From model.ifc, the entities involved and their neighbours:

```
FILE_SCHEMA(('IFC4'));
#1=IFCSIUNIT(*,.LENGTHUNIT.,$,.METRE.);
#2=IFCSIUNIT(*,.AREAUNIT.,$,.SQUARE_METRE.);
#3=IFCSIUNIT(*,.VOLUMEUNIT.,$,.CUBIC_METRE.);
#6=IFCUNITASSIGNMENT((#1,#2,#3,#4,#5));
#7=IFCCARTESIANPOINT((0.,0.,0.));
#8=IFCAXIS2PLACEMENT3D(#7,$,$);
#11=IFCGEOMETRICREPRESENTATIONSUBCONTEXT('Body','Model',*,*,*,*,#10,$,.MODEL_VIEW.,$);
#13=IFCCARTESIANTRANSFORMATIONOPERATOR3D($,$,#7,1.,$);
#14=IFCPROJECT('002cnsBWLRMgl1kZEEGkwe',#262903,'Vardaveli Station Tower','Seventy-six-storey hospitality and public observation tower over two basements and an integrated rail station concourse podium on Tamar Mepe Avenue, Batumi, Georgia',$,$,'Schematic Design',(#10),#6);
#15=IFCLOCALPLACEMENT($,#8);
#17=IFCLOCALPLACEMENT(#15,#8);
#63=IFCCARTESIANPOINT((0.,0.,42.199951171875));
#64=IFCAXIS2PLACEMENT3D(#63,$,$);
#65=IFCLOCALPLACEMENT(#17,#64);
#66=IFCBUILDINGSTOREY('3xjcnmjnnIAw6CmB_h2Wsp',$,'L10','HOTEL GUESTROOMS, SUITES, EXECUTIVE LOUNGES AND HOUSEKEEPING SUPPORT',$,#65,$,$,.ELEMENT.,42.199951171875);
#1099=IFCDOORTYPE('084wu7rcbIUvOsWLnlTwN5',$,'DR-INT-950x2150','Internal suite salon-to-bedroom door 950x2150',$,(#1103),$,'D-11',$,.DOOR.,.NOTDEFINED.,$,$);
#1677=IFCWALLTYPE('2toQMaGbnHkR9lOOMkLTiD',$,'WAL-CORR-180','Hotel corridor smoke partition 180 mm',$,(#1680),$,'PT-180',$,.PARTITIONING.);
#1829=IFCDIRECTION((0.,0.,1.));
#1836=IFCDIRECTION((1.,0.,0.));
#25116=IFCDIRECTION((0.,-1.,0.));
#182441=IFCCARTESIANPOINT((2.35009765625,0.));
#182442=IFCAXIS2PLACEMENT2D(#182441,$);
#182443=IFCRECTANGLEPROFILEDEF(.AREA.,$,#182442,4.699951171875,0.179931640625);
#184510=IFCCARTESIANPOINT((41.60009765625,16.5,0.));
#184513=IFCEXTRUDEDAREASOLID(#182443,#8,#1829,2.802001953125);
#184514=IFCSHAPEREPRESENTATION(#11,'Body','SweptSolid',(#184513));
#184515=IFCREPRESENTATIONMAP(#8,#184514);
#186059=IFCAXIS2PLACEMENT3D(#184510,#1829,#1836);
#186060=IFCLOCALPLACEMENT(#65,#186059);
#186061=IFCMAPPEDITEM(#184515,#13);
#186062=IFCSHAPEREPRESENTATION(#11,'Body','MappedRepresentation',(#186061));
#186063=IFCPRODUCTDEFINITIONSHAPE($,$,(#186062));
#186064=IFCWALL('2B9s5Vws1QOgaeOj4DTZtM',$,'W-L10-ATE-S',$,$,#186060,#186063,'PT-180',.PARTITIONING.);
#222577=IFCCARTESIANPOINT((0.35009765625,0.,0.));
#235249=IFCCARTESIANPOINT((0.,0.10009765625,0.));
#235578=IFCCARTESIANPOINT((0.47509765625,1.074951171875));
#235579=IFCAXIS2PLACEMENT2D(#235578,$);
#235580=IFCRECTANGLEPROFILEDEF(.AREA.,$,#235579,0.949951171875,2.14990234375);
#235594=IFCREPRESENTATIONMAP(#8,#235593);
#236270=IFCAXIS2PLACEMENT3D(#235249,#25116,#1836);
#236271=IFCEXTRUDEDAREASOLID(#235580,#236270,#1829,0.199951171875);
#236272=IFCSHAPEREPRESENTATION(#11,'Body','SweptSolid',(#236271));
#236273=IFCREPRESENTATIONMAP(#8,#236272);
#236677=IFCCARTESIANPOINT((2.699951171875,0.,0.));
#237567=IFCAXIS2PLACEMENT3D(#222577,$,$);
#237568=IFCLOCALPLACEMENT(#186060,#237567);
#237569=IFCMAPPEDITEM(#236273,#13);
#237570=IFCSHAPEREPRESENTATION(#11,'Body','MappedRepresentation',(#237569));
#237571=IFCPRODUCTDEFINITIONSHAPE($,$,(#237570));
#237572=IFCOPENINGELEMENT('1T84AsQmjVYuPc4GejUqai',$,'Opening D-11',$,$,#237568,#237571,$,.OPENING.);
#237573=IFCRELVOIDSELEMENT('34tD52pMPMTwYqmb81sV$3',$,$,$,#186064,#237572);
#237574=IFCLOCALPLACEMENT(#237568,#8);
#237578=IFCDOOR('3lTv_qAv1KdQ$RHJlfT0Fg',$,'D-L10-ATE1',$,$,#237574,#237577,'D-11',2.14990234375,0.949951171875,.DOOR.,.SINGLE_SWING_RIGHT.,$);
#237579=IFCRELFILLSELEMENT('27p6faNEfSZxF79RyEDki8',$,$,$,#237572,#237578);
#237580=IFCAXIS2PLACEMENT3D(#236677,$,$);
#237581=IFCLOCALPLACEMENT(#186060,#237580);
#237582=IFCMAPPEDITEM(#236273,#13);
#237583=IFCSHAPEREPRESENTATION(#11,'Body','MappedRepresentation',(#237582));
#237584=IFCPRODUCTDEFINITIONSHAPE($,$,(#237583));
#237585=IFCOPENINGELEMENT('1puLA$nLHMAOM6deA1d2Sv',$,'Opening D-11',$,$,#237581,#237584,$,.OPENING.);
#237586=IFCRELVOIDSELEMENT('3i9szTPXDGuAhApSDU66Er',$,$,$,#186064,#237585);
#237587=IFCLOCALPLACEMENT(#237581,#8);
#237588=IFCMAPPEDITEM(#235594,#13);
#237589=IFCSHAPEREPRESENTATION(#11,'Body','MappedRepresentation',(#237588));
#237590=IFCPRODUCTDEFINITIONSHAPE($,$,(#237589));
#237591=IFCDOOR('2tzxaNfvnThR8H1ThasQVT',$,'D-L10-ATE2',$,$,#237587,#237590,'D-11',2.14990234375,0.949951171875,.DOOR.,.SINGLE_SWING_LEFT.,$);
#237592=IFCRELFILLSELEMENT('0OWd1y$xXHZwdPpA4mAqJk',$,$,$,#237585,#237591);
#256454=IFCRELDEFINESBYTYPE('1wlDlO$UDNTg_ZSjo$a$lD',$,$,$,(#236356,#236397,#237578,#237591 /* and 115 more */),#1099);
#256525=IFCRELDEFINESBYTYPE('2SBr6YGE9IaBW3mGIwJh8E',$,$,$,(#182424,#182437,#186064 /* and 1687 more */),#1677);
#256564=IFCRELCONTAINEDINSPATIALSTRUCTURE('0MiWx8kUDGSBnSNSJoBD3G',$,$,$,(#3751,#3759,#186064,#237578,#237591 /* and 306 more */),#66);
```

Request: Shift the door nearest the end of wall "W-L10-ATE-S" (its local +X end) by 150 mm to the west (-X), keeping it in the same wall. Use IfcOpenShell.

```python
import ifcopenshell
import ifcopenshell.api.geometry
import ifcopenshell.util.placement
import ifcopenshell.util.unit

model = ifcopenshell.open("model.ifc")
unit_scale = ifcopenshell.util.unit.calculate_unit_scale(model)

door = model.by_guid("2tzxaNfvnThR8H1ThasQVT")
opening = door.FillsVoids[0].RelatingOpeningElement
wall = opening.VoidsElements[0].RelatingBuildingElement

wall_matrix = ifcopenshell.util.placement.get_local_placement(wall.ObjectPlacement)
shift = wall_matrix[:3, 0] * -0.15 / unit_scale
before = ifcopenshell.util.placement.get_local_placement(door.ObjectPlacement)[:3, 3].copy()

# The door is placed relative to its opening, so it follows when the opening moves.
matrix = ifcopenshell.util.placement.get_local_placement(opening.ObjectPlacement)
matrix[:3, 3] += shift
ifcopenshell.api.geometry.edit_object_placement(
    model, product=opening, matrix=matrix, is_si=False, should_transform_children=True
)

after = ifcopenshell.util.placement.get_local_placement(door.ObjectPlacement)[:3, 3]
print("door moved by", (after - before).round(3) + 0.0)

model.write("model_updated.ifc")
```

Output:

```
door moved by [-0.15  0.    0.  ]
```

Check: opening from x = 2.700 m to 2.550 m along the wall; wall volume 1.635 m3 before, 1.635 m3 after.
